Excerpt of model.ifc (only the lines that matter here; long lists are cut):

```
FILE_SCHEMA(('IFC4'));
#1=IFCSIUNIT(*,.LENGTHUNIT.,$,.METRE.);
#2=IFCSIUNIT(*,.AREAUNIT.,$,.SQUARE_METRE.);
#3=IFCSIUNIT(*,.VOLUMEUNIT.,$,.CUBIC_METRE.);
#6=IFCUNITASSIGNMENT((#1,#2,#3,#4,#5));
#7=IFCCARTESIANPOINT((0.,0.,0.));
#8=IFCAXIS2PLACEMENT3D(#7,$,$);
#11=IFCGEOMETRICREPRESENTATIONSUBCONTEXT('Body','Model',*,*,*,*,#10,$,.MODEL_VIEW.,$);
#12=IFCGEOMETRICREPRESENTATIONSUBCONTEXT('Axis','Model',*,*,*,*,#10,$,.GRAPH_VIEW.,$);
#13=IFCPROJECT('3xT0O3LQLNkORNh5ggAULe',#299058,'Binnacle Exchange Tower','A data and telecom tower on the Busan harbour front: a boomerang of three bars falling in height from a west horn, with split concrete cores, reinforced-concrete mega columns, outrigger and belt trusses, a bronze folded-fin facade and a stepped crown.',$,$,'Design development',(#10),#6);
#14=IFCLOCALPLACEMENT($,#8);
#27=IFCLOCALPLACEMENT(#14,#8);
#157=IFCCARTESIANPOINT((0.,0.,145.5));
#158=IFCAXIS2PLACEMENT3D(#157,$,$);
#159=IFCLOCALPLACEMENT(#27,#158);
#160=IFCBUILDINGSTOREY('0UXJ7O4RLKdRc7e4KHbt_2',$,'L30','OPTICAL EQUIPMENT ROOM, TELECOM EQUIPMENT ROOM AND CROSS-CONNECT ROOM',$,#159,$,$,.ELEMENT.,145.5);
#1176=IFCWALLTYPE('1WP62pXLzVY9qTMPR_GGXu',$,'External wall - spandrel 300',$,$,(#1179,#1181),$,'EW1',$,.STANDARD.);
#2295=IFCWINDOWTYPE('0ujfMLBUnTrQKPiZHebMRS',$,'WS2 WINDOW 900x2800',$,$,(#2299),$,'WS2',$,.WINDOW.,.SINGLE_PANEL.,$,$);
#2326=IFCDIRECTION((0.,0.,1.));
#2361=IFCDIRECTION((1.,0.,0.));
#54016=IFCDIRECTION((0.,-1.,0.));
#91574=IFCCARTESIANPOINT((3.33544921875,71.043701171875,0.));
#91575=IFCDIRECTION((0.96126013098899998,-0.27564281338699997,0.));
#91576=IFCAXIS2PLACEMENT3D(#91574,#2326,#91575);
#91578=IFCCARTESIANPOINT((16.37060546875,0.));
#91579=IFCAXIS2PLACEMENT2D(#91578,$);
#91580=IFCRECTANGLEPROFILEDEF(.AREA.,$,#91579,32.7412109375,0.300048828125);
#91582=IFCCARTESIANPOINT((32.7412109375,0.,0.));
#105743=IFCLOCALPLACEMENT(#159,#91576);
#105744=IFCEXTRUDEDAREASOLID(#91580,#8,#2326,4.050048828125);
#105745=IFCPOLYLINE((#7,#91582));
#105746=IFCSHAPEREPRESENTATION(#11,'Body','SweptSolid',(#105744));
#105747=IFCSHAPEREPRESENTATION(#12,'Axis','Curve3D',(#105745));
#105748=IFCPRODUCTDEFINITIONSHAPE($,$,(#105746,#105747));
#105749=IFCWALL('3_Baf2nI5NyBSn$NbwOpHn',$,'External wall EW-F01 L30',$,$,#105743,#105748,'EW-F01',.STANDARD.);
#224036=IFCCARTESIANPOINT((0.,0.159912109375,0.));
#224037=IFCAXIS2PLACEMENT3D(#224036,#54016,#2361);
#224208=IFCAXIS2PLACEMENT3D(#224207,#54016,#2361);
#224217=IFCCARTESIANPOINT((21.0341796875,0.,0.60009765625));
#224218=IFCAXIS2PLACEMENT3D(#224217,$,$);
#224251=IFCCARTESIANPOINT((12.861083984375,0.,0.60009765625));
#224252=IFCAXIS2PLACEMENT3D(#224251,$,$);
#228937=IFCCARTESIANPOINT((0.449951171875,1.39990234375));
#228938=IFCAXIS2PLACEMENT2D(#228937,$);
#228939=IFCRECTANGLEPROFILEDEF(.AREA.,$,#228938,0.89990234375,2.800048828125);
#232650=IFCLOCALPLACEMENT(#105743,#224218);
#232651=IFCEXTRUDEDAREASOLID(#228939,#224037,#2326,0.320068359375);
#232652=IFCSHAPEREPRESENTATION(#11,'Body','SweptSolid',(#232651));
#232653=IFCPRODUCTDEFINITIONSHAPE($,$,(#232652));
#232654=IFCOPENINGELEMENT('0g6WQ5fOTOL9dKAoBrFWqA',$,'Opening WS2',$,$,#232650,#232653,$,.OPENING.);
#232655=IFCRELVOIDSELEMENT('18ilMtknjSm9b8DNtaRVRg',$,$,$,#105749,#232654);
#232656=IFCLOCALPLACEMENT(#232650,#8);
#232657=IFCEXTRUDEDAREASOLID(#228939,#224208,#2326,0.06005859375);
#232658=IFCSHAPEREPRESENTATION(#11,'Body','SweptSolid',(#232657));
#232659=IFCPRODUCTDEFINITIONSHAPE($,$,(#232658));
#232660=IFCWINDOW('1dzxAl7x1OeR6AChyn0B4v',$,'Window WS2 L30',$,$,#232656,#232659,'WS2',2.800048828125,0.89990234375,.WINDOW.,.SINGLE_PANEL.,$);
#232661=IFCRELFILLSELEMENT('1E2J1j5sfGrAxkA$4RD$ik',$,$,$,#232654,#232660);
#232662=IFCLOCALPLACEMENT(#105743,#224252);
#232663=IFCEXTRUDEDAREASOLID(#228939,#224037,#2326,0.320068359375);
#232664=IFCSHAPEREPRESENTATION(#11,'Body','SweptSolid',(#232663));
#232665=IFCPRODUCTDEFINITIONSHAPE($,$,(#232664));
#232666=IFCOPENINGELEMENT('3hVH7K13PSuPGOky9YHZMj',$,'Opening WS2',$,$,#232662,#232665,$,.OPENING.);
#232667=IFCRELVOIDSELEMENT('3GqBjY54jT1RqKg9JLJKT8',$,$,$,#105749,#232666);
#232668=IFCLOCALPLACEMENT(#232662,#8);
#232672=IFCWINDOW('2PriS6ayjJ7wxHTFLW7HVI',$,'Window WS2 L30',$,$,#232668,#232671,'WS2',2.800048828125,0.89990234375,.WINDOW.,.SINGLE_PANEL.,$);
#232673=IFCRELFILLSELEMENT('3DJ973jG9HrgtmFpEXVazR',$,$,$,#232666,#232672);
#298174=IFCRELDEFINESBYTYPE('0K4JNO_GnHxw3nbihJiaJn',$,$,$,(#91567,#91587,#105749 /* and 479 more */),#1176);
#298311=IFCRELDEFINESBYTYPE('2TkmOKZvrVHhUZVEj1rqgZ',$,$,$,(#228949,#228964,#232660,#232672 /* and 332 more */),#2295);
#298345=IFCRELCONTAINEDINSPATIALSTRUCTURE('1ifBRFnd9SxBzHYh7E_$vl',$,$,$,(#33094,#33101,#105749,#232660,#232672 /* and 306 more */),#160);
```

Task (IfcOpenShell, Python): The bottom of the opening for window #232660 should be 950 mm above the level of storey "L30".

```python
import numpy as np
import ifcopenshell
import ifcopenshell.api.geometry
import ifcopenshell.geom
import ifcopenshell.util.element
import ifcopenshell.util.placement
import ifcopenshell.util.shape
import ifcopenshell.util.unit

model = ifcopenshell.open("model.ifc")
unit_scale = ifcopenshell.util.unit.calculate_unit_scale(model)

window = model.by_id(232660)
opening = window.FillsVoids[0].RelatingOpeningElement
storey = ifcopenshell.util.element.get_container(window, ifc_class="IfcBuildingStorey")
level = ifcopenshell.util.placement.get_local_placement(storey.ObjectPlacement)[2, 3]

# The opening's origin need not be at the sill, so measure its lowest point.
shape = ifcopenshell.geom.create_shape(ifcopenshell.geom.settings(), opening)
bottom = ifcopenshell.util.shape.get_shape_bottom_elevation(shape, shape.geometry) / unit_scale
dz = level + 0.95 - bottom

shift = np.array([0.0, 0.0, dz])
# The window is placed relative to its opening, so it follows when the opening moves.
matrix = ifcopenshell.util.placement.get_local_placement(opening.ObjectPlacement)
matrix[:3, 3] += shift
ifcopenshell.api.geometry.edit_object_placement(
    model, product=opening, matrix=matrix, is_si=False, should_transform_children=True
)

print(f"moved by {dz * unit_scale:+.3f} m")

model.write("model_updated.ifc")
```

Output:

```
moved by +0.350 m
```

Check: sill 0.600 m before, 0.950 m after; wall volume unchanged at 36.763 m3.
